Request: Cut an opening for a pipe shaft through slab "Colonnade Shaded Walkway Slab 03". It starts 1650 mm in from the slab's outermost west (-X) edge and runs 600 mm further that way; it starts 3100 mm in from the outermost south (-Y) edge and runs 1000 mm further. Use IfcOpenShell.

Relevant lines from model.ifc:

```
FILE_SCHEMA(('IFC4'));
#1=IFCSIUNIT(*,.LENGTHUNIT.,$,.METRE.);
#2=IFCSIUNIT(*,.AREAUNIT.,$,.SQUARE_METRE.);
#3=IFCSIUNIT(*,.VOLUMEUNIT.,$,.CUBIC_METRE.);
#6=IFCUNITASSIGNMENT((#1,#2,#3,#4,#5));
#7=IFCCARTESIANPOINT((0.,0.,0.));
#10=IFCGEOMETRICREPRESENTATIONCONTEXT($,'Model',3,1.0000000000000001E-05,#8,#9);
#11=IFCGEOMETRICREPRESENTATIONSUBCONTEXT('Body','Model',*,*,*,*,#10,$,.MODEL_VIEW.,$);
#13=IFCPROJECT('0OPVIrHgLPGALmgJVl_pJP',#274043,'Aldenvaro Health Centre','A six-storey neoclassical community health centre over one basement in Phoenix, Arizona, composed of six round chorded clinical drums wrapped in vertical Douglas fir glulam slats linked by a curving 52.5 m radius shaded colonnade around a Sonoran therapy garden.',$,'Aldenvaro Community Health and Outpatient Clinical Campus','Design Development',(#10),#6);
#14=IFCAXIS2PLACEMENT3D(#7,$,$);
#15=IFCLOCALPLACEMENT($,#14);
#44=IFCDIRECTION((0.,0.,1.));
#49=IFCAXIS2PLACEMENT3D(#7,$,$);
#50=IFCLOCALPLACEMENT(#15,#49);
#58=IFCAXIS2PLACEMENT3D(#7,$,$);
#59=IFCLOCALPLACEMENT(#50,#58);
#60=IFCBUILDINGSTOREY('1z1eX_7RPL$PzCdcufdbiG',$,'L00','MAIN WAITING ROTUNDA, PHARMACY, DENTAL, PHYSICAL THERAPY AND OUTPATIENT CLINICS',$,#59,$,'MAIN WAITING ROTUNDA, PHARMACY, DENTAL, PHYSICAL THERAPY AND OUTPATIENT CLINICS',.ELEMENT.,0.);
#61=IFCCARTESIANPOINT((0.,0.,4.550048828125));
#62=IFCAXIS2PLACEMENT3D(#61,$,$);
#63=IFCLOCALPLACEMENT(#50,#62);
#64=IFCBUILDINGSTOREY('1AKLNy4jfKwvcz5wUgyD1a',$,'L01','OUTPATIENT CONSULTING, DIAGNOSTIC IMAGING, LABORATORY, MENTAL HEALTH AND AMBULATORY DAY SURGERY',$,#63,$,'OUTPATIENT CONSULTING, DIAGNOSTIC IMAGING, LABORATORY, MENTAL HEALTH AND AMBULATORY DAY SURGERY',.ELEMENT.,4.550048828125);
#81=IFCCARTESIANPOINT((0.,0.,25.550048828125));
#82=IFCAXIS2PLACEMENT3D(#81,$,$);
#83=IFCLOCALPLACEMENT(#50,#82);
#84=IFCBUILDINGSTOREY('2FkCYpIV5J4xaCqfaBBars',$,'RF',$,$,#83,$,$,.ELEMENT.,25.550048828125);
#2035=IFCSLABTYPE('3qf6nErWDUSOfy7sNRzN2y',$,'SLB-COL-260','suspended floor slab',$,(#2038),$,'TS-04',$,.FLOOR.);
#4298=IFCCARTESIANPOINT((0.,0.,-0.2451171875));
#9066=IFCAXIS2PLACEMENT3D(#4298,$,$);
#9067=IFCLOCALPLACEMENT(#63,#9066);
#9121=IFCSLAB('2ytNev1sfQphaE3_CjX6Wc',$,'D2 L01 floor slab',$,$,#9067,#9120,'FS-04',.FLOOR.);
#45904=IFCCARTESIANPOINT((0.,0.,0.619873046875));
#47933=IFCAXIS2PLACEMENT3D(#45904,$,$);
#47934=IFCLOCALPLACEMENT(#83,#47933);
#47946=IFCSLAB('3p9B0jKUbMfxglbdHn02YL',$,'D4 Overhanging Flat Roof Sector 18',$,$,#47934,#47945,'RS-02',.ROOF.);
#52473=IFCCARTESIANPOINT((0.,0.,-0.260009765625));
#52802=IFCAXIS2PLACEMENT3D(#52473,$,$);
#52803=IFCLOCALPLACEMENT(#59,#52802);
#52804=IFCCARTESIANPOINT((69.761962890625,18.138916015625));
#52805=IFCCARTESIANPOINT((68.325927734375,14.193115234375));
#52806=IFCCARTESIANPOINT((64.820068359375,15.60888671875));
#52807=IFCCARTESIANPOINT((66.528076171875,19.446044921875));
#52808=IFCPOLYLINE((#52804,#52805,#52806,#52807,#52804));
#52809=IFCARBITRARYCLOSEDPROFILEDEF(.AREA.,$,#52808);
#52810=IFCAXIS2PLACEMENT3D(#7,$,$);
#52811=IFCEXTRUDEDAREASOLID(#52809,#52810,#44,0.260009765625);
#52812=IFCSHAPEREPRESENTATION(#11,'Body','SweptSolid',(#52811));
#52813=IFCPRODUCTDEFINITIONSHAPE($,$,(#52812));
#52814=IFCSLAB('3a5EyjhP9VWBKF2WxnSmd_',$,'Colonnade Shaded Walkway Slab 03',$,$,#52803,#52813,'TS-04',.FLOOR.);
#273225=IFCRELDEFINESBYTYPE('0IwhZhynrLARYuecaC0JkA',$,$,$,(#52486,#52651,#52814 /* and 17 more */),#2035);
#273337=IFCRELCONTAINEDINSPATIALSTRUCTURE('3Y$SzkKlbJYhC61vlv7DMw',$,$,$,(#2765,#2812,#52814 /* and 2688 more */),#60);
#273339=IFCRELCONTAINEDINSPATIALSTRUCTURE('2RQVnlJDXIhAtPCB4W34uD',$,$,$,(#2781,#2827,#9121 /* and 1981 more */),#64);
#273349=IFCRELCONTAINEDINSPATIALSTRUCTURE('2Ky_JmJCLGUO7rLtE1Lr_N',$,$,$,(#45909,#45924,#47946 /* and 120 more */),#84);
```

```python
import numpy as np
import ifcopenshell
import ifcopenshell.api.feature
import ifcopenshell.api.geometry
import ifcopenshell.api.root
import ifcopenshell.geom
import ifcopenshell.util.placement
import ifcopenshell.util.representation
import ifcopenshell.util.shape
import ifcopenshell.util.unit

model = ifcopenshell.open("model.ifc")
unit_scale = ifcopenshell.util.unit.calculate_unit_scale(model)
settings = ifcopenshell.geom.settings()


def volume(element):
    """Net volume in cubic metres, openings subtracted."""
    shape = ifcopenshell.geom.create_shape(settings, element)
    return ifcopenshell.util.shape.get_volume(shape.geometry)


slab = model.by_id(52814)
before = volume(slab)

# Extent in the slab's own axes, in metres. The edges named are its -X and -Y sides.
slab_shape = ifcopenshell.geom.create_shape(settings, slab)
vertices = ifcopenshell.util.shape.get_vertices(slab_shape.geometry)
x_min, y_min, bottom = vertices.min(axis=0)
top = vertices[:, 2].max()

opening = ifcopenshell.api.root.create_entity(model, ifc_class="IfcOpeningElement", name="Pipe shaft opening", predefined_type="OPENING")
context = ifcopenshell.util.representation.get_context(model, "Model", "Body", "MODEL_VIEW")
width, depth = 0.6, 1
outline = [(0.0, 0.0), (width, 0.0), (width, depth), (0.0, depth), (0.0, 0.0)]
# Overshoot both faces by 50 mm so the cut is clean.
shape = ifcopenshell.api.geometry.add_slab_representation(
    model, context=context, depth=top - bottom + 0.1, polyline=outline
)
ifcopenshell.api.geometry.assign_representation(model, product=opening, representation=shape)

matrix = ifcopenshell.util.placement.get_local_placement(slab.ObjectPlacement)
matrix[:, 3] = matrix @ np.append(np.array([x_min + 1.65, y_min + 3.1, bottom - 0.05]) / unit_scale, 1.0)
ifcopenshell.api.geometry.edit_object_placement(model, product=opening, matrix=matrix, is_si=False)
ifcopenshell.api.feature.add_feature(model, feature=opening, element=slab)

after = volume(slab)

print(f"slab volume {before:.3f} -> {after:.3f} m3")

model.write("model_v2.ifc")
```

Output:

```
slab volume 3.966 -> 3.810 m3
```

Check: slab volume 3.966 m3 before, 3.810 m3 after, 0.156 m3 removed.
